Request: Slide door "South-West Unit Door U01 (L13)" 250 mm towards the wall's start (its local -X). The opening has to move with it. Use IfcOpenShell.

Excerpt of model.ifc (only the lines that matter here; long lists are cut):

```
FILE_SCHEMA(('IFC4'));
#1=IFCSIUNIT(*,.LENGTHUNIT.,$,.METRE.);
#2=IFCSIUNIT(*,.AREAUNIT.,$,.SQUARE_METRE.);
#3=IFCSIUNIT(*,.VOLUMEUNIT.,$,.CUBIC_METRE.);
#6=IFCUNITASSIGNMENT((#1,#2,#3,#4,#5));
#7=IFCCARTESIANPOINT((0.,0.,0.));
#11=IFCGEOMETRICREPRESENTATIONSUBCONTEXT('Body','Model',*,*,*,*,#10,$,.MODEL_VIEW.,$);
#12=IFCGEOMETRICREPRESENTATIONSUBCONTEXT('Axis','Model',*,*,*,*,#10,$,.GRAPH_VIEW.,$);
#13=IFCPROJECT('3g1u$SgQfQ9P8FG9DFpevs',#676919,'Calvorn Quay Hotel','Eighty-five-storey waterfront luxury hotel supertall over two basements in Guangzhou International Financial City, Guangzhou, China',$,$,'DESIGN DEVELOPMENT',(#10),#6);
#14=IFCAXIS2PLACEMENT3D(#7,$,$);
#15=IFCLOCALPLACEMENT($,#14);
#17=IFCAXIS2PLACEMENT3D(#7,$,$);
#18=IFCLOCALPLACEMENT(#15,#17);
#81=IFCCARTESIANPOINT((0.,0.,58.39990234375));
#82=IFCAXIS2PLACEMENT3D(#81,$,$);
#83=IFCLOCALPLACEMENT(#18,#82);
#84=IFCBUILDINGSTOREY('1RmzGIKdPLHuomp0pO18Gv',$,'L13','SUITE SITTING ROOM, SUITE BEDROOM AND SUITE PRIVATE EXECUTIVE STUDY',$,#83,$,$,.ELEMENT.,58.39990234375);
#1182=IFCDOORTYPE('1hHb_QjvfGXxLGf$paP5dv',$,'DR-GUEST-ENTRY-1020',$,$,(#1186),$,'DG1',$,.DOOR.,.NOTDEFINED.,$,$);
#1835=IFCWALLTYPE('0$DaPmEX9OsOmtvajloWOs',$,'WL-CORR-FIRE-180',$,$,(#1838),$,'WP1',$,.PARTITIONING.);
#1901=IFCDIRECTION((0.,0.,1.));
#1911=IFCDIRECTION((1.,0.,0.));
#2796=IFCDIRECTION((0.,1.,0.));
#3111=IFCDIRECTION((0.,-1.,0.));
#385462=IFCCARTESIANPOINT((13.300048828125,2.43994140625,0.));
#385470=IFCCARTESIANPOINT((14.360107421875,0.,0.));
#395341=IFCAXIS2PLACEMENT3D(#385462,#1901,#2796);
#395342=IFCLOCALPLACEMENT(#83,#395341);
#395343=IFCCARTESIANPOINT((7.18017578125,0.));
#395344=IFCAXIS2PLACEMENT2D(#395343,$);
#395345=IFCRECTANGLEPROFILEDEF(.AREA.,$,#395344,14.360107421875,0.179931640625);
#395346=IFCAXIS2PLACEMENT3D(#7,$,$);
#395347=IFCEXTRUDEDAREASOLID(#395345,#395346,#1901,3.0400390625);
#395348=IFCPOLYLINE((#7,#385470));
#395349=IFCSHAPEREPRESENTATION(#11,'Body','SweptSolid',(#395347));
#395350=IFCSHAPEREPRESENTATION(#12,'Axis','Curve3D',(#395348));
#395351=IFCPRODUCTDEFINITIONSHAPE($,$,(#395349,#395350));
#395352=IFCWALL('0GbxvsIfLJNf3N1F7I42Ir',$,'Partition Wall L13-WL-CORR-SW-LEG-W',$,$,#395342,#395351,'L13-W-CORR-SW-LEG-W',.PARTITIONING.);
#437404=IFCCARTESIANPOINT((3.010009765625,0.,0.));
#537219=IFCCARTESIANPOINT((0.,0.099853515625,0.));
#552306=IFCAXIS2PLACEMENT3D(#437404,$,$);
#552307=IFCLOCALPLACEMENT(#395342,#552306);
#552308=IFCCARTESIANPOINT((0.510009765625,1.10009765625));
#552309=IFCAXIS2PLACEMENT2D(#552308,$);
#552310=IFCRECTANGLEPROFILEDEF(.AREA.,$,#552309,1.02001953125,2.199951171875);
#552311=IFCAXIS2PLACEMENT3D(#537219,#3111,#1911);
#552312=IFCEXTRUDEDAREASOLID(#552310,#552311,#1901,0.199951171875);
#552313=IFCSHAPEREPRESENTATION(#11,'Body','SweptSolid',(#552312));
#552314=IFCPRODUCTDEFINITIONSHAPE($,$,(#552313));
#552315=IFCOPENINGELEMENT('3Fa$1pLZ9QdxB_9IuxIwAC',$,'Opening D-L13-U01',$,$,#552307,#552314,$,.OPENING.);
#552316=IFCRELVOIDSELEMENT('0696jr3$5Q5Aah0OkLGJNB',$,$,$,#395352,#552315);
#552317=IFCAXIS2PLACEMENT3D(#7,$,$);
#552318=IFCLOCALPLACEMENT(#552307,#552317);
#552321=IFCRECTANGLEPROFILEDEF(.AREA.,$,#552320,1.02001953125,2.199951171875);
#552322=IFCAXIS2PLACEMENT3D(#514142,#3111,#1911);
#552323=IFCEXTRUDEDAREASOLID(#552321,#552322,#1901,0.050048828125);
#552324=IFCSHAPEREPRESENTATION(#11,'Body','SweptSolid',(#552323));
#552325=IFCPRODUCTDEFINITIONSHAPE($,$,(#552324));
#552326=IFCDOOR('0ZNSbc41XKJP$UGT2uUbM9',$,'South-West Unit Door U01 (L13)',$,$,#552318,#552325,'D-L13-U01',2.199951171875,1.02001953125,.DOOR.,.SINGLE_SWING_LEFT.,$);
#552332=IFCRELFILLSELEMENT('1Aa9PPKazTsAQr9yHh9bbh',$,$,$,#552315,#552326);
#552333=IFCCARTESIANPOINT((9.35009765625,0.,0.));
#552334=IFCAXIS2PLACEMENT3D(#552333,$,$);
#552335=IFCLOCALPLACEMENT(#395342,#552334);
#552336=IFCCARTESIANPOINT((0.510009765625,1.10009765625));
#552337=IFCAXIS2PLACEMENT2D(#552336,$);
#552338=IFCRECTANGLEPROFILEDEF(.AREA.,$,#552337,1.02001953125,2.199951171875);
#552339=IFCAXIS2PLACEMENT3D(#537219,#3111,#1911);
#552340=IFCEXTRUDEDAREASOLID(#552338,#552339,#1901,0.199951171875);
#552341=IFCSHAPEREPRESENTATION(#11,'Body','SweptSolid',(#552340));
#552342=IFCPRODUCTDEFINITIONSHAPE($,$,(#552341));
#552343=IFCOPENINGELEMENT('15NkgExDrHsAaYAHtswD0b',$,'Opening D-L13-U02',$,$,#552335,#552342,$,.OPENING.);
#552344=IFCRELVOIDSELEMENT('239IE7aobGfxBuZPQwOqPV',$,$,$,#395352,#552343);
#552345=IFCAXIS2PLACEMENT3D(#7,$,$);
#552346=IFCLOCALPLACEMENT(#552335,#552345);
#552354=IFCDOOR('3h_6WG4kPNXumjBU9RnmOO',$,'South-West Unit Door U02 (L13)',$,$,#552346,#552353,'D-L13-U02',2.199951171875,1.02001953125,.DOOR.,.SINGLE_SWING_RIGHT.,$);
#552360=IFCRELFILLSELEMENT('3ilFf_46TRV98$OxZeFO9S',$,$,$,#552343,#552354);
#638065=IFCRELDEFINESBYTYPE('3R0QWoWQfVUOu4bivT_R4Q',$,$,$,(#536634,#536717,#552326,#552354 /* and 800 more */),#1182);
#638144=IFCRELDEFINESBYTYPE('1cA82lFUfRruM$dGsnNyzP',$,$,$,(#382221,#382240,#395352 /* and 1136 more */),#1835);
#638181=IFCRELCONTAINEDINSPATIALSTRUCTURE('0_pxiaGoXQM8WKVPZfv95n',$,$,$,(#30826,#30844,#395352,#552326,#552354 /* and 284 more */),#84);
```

```python
import ifcopenshell
import ifcopenshell.api.geometry
import ifcopenshell.util.placement
import ifcopenshell.util.unit

model = ifcopenshell.open("model.ifc")
unit_scale = ifcopenshell.util.unit.calculate_unit_scale(model)

door = model.by_guid("0ZNSbc41XKJP$UGT2uUbM9")
opening = door.FillsVoids[0].RelatingOpeningElement
wall = opening.VoidsElements[0].RelatingBuildingElement

wall_matrix = ifcopenshell.util.placement.get_local_placement(wall.ObjectPlacement)
shift = wall_matrix[:3, 0] * -0.25 / unit_scale
before = ifcopenshell.util.placement.get_local_placement(door.ObjectPlacement)[:3, 3].copy()

# The door is placed relative to its opening, so it follows when the opening moves.
matrix = ifcopenshell.util.placement.get_local_placement(opening.ObjectPlacement)
matrix[:3, 3] += shift
ifcopenshell.api.geometry.edit_object_placement(
    model, product=opening, matrix=matrix, is_si=False, should_transform_children=True
)

after = ifcopenshell.util.placement.get_local_placement(door.ObjectPlacement)[:3, 3]
print("door moved by", (after - before).round(3) + 0.0)

model.write("model_edited.ifc")
```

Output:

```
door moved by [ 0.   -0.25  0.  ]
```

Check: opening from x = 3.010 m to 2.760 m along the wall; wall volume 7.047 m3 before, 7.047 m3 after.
